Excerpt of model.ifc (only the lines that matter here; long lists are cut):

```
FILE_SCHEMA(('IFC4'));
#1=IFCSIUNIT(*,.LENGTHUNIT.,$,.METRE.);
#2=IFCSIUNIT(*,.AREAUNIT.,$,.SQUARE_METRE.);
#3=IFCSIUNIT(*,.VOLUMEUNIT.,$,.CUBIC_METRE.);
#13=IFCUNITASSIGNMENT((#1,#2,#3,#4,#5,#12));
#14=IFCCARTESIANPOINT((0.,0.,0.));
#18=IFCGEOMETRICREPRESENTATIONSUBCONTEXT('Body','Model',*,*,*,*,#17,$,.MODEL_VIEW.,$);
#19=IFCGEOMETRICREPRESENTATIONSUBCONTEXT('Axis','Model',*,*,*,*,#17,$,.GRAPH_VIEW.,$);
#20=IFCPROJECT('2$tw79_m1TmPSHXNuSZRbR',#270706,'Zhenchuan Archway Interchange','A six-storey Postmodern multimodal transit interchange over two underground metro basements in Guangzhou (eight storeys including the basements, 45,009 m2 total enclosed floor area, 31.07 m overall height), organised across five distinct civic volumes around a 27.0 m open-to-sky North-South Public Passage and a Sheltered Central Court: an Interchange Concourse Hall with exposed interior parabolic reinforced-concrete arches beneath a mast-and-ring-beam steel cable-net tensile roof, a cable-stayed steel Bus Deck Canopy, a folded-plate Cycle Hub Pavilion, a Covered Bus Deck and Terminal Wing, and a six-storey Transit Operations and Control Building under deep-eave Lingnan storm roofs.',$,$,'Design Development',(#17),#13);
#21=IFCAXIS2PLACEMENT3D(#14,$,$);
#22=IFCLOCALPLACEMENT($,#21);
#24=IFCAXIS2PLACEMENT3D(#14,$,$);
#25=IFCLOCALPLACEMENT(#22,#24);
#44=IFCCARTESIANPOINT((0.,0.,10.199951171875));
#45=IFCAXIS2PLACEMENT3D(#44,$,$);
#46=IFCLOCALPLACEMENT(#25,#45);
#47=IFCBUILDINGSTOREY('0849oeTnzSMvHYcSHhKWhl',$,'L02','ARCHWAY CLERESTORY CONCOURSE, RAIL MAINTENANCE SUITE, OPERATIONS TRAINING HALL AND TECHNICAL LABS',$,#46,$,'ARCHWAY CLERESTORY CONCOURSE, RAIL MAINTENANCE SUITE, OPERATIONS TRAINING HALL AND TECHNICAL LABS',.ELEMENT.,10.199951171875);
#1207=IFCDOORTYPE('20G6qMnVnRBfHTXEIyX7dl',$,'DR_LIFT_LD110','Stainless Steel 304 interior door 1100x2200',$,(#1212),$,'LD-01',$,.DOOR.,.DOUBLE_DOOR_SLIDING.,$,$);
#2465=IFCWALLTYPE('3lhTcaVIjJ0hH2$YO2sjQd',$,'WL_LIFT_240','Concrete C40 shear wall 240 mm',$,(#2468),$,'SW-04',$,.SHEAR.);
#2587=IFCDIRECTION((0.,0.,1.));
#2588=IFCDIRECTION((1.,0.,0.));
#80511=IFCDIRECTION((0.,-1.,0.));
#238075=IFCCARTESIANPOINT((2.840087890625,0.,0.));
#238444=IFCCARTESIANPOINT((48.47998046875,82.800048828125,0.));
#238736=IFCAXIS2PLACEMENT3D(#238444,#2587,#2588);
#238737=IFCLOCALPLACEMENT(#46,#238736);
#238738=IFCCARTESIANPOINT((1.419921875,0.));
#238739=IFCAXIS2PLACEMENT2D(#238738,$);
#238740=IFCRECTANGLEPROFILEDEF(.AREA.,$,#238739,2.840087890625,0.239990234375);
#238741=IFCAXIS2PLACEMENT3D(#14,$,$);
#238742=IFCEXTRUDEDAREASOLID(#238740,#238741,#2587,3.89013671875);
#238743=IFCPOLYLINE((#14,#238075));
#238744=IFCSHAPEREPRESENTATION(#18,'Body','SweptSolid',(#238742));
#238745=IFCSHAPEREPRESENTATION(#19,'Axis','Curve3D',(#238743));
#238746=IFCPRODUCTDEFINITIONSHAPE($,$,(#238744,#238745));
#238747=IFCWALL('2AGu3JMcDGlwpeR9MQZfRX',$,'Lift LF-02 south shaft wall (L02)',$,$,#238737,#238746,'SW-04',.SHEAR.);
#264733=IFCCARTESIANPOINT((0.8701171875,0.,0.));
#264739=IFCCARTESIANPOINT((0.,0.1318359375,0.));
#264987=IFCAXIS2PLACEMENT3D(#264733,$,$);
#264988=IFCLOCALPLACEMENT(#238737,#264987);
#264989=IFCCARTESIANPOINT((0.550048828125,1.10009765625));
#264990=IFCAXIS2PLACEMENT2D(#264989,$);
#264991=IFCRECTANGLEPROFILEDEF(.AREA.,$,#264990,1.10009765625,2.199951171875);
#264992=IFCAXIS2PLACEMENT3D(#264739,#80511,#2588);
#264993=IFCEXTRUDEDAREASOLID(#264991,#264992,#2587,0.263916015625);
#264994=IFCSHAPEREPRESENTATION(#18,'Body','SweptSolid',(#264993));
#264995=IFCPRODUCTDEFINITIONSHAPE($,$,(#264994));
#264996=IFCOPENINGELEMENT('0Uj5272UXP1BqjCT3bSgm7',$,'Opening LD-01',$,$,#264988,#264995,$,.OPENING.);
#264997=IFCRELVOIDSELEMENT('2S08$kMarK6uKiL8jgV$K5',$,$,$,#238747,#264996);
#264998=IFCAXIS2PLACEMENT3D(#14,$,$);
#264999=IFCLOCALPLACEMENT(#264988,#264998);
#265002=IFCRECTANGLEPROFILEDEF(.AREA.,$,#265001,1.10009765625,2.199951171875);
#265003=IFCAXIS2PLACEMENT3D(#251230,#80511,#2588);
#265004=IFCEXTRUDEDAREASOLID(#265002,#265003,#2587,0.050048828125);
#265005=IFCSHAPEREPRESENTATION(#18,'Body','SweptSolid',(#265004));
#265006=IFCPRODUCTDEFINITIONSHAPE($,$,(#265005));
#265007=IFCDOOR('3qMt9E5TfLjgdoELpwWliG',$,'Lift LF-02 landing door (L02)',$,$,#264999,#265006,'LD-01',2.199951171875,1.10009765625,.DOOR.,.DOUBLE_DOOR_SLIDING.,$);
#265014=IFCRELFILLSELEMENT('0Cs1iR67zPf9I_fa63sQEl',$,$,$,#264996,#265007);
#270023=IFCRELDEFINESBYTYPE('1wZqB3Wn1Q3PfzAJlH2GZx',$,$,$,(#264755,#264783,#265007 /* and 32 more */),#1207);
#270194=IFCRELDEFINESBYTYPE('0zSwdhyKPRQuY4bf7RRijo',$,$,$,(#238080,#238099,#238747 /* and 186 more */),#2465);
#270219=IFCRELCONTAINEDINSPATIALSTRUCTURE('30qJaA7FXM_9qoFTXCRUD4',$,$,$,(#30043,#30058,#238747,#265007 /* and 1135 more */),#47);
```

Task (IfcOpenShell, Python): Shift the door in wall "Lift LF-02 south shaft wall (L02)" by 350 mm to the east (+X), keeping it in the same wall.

```python
import ifcopenshell
import ifcopenshell.api.geometry
import ifcopenshell.util.placement

model = ifcopenshell.open("model.ifc")

door = model.by_id(265007)
opening = door.FillsVoids[0].RelatingOpeningElement
wall = opening.VoidsElements[0].RelatingBuildingElement

wall_matrix = ifcopenshell.util.placement.get_local_placement(wall.ObjectPlacement)
shift = wall_matrix[:3, 0] * 0.35
before = ifcopenshell.util.placement.get_local_placement(door.ObjectPlacement)[:3, 3].copy()

# The door is placed relative to its opening, so it follows when the opening moves.
matrix = ifcopenshell.util.placement.get_local_placement(opening.ObjectPlacement)
matrix[:3, 3] += shift
ifcopenshell.api.geometry.edit_object_placement(
    model, product=opening, matrix=matrix, is_si=False, should_transform_children=True
)

after = ifcopenshell.util.placement.get_local_placement(door.ObjectPlacement)[:3, 3]
print("door moved by", (after - before).round(3) + 0.0)

model.write("model_edited.ifc")
```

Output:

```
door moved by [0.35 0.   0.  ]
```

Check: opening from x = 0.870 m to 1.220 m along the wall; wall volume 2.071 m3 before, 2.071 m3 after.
